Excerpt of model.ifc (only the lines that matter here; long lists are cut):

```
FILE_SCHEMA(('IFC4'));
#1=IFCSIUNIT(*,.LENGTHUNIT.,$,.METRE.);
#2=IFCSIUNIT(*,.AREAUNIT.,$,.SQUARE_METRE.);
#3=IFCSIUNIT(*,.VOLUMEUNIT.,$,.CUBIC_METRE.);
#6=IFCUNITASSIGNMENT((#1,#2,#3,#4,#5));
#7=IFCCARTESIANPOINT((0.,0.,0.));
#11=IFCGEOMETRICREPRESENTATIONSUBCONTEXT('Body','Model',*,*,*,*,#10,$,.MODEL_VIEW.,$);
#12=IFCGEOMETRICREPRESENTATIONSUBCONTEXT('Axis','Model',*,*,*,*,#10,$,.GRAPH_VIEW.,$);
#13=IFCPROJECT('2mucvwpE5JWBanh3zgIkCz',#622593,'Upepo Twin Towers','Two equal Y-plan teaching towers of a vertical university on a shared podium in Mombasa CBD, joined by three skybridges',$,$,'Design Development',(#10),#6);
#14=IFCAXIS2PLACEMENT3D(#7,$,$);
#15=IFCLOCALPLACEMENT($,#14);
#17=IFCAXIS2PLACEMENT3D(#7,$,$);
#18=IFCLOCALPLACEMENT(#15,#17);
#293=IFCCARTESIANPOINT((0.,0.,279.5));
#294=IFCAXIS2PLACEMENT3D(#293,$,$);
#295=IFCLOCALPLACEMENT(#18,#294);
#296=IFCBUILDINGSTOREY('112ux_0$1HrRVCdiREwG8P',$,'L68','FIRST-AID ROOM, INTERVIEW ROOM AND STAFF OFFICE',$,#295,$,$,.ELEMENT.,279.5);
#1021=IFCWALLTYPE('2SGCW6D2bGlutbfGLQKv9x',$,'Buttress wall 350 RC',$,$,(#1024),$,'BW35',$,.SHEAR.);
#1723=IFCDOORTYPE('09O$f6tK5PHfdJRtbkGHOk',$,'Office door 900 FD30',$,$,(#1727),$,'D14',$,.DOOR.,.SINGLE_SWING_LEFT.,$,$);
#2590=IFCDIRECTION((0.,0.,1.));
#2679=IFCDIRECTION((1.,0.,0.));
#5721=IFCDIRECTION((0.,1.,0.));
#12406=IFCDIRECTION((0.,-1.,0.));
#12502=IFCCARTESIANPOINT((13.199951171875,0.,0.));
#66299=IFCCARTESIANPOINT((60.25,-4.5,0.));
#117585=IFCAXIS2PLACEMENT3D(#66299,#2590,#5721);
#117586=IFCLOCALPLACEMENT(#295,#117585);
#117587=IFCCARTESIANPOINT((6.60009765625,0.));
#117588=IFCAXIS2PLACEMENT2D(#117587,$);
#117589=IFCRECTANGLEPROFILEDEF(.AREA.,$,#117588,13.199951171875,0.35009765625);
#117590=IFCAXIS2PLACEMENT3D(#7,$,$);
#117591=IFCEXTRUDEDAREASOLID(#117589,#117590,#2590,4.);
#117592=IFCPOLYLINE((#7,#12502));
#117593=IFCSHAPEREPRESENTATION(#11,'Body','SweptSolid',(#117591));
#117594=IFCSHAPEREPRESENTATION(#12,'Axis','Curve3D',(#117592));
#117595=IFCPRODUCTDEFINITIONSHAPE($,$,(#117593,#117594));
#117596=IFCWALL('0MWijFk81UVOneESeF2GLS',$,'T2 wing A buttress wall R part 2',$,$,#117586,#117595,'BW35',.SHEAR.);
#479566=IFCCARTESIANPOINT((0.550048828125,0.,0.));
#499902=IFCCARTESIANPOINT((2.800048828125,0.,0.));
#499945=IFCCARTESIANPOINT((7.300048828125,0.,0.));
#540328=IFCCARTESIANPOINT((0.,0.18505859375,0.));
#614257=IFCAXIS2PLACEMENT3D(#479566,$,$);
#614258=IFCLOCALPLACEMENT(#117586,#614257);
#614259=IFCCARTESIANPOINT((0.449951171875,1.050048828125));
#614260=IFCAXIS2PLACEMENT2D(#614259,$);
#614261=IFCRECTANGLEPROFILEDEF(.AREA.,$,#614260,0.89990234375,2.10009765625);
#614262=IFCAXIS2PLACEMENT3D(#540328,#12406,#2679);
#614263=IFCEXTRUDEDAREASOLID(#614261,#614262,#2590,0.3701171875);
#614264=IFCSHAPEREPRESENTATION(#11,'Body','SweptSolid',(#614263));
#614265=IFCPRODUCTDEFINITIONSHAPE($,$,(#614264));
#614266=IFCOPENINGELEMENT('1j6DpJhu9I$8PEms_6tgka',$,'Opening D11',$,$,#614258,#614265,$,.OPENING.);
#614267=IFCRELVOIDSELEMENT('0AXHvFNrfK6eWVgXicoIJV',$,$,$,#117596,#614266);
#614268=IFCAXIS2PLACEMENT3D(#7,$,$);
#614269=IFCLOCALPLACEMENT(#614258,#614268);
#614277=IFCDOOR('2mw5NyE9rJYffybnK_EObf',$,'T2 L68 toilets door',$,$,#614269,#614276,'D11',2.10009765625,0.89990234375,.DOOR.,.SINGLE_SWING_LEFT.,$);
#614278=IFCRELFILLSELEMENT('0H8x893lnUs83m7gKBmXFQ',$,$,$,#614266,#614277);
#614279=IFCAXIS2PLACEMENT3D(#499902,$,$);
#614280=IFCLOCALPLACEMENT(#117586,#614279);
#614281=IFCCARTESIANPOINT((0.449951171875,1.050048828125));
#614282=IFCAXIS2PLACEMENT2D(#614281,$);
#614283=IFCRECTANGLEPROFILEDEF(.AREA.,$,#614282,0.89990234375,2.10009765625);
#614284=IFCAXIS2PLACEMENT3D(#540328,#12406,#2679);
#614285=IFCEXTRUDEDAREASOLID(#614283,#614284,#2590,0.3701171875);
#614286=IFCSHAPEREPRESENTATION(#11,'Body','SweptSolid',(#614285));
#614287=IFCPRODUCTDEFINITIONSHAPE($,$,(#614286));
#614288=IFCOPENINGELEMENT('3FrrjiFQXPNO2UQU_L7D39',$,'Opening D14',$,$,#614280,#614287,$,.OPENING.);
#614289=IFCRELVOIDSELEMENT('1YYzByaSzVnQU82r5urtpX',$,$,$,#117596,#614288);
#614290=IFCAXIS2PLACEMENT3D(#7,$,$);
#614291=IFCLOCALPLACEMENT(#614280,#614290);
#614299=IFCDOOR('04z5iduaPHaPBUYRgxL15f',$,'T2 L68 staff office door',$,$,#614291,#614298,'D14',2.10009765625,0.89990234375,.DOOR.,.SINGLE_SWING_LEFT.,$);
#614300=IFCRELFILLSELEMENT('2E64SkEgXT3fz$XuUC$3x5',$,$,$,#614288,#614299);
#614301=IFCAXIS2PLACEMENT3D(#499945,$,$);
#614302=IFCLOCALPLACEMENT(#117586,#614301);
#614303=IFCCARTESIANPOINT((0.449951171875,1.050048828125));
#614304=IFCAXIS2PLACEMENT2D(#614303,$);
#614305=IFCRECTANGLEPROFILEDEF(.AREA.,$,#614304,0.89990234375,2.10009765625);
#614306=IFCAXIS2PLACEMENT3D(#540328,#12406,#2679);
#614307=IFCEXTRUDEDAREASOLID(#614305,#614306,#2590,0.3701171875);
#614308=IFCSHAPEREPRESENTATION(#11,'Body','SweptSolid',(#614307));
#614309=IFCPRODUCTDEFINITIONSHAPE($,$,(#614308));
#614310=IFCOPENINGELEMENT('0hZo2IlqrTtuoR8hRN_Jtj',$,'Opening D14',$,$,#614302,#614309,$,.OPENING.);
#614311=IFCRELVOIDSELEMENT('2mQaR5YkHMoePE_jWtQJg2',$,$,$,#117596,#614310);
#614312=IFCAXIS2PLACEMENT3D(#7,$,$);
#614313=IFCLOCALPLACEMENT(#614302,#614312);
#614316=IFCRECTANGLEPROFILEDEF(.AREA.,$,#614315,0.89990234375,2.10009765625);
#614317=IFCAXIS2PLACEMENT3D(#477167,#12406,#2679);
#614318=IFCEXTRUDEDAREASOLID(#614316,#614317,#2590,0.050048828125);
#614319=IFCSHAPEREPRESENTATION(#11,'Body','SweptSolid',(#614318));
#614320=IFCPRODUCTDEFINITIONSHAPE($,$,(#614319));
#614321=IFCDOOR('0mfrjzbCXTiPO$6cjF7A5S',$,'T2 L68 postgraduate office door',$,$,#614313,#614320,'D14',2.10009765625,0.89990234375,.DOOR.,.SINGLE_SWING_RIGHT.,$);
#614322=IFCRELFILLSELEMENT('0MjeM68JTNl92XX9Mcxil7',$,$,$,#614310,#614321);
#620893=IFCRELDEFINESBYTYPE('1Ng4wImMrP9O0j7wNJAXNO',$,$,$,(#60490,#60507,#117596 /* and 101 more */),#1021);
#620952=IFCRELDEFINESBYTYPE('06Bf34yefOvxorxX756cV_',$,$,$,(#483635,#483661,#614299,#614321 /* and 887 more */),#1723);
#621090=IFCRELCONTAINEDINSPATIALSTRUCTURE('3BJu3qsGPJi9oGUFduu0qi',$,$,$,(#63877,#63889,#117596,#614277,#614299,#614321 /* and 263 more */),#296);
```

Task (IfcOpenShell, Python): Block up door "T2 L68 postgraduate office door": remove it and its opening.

```python
import ifcopenshell
import ifcopenshell.api.feature
import ifcopenshell.api.root
import ifcopenshell.geom
import ifcopenshell.util.shape

model = ifcopenshell.open("model.ifc")
settings = ifcopenshell.geom.settings()


def volume(element):
    """Net volume in cubic metres, openings subtracted."""
    shape = ifcopenshell.geom.create_shape(settings, element)
    return ifcopenshell.util.shape.get_volume(shape.geometry)


door = model.by_guid("0mfrjzbCXTiPO$6cjF7A5S")
opening = door.FillsVoids[0].RelatingOpeningElement
wall = opening.VoidsElements[0].RelatingBuildingElement
before = volume(wall)

ifcopenshell.api.root.remove_product(model, product=door)
ifcopenshell.api.feature.remove_feature(model, feature=opening)

after = volume(wall)

print(f"wall volume {before:.3f} -> {after:.3f} m3")

model.write("model-out.ifc")
```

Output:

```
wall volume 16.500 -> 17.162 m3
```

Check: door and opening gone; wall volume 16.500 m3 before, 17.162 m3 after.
